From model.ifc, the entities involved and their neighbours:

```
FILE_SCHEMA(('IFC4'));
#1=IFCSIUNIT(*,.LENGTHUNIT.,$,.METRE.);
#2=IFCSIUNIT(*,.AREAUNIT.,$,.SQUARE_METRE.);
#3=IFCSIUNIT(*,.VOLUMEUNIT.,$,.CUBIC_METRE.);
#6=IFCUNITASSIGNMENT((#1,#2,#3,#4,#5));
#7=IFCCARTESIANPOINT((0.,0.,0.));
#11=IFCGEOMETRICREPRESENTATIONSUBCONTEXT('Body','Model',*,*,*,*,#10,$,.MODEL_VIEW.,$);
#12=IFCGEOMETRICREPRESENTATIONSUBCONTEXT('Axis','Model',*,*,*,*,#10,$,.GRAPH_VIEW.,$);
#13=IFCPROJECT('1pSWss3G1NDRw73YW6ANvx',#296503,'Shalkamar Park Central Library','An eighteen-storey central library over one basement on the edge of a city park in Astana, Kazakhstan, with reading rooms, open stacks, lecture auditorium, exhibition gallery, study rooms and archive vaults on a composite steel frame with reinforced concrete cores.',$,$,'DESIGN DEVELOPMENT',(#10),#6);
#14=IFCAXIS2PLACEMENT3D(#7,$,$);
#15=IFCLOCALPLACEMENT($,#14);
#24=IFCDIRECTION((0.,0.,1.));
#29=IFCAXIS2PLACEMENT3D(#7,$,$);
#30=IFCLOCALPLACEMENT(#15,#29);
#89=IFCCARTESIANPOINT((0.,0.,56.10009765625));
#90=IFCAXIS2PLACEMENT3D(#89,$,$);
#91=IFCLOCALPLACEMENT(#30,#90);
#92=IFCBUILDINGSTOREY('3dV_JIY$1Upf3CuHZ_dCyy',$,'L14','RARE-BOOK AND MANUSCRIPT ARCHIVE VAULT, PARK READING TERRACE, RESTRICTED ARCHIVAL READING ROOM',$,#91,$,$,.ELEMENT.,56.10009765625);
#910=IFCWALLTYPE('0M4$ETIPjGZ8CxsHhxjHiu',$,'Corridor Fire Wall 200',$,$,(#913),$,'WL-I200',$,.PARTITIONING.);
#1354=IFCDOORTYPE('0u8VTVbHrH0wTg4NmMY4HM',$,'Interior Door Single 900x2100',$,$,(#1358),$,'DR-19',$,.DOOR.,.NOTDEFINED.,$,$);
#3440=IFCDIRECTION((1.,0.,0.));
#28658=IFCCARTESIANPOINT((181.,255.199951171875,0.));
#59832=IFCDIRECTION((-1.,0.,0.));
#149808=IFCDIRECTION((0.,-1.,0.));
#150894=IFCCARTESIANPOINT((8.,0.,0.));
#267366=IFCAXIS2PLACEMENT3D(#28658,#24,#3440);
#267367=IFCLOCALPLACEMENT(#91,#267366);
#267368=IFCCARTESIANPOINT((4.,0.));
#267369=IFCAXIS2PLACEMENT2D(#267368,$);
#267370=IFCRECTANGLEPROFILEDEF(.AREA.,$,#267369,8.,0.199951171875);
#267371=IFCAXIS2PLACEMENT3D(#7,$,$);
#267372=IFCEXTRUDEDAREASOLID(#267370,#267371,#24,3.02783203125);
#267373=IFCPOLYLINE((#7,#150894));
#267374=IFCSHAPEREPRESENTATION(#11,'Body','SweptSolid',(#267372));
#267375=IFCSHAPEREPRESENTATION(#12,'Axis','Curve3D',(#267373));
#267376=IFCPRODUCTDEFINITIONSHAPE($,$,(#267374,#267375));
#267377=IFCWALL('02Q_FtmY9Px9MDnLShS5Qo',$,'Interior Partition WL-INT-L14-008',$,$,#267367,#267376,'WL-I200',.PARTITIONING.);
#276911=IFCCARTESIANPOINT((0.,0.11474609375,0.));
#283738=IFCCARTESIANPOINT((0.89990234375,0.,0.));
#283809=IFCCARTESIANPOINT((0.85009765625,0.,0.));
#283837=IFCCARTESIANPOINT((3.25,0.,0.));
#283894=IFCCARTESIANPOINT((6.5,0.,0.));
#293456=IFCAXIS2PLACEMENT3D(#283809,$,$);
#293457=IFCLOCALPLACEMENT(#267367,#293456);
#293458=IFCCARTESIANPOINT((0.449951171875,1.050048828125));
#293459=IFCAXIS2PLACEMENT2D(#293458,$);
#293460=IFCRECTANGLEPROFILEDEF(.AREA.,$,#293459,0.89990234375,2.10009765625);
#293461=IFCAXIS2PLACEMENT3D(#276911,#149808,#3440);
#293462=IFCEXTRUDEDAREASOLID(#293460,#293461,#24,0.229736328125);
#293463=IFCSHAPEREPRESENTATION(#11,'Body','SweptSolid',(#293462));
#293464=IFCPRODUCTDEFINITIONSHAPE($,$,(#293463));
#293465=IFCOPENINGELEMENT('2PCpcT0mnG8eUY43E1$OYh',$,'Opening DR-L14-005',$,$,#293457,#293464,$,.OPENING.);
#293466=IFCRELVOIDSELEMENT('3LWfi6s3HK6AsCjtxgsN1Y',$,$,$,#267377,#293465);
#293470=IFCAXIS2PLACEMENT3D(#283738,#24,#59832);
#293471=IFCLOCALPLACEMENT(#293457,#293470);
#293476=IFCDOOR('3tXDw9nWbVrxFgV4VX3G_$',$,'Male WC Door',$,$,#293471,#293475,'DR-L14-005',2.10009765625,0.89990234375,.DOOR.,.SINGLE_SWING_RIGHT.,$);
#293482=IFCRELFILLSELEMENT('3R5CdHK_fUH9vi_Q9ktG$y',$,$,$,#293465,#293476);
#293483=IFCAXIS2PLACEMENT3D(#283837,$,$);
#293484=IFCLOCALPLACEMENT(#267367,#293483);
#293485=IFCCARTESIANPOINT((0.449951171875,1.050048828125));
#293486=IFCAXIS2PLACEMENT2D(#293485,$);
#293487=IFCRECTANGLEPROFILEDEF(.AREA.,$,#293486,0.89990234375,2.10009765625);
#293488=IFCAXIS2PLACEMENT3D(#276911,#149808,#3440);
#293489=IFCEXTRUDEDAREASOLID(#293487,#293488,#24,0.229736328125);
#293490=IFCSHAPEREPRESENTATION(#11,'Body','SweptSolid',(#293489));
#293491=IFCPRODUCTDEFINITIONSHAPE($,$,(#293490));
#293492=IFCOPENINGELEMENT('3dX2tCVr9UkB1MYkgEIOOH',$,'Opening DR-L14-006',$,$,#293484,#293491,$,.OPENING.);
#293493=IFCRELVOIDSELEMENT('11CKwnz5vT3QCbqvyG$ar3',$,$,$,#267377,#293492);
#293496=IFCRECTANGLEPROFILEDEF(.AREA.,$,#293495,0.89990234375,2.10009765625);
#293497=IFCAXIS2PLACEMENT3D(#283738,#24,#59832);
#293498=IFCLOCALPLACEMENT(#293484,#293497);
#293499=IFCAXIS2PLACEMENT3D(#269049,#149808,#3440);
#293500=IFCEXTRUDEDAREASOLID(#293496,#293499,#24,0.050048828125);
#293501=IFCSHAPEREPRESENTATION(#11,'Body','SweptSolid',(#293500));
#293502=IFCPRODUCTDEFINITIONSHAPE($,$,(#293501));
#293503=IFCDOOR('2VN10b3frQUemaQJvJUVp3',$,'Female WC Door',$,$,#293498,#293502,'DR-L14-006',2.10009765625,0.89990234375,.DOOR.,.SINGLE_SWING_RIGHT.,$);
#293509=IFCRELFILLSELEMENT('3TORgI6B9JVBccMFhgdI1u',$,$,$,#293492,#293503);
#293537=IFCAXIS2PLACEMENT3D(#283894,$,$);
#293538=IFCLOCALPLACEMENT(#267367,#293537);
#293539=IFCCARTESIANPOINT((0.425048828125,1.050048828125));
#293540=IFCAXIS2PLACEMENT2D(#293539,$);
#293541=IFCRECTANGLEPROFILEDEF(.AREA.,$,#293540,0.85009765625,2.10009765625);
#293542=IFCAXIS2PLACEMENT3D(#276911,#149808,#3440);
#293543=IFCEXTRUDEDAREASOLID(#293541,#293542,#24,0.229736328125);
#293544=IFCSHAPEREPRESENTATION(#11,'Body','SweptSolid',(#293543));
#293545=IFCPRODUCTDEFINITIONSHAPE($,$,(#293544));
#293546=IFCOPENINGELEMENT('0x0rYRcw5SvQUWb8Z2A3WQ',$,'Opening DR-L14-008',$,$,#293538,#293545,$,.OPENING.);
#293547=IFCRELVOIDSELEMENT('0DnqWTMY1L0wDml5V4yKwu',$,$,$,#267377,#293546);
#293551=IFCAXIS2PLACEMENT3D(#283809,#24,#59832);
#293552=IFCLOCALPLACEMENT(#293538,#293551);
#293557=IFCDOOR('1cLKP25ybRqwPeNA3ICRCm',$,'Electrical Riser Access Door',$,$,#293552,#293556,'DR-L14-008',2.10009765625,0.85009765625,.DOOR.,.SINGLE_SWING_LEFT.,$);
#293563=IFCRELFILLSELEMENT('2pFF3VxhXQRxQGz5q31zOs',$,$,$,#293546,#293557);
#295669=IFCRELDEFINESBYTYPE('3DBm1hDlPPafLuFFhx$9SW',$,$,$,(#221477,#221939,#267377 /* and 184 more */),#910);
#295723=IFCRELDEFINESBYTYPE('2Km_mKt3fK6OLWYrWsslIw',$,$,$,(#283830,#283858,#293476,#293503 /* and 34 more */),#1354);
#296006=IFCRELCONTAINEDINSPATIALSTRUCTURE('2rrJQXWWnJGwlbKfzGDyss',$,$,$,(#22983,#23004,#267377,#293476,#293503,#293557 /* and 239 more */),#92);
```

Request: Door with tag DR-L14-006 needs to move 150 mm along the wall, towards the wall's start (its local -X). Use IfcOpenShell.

```python
import ifcopenshell
import ifcopenshell.api.geometry
import ifcopenshell.util.placement

model = ifcopenshell.open("model.ifc")

door = model.by_guid("2VN10b3frQUemaQJvJUVp3")
opening = door.FillsVoids[0].RelatingOpeningElement
wall = opening.VoidsElements[0].RelatingBuildingElement

wall_matrix = ifcopenshell.util.placement.get_local_placement(wall.ObjectPlacement)
shift = wall_matrix[:3, 0] * -0.15
before = ifcopenshell.util.placement.get_local_placement(door.ObjectPlacement)[:3, 3].copy()

# The door is placed relative to its opening, so it follows when the opening moves.
matrix = ifcopenshell.util.placement.get_local_placement(opening.ObjectPlacement)
matrix[:3, 3] += shift
ifcopenshell.api.geometry.edit_object_placement(
    model, product=opening, matrix=matrix, is_si=False, should_transform_children=True
)

after = ifcopenshell.util.placement.get_local_placement(door.ObjectPlacement)[:3, 3]
print("door moved by", (after - before).round(3) + 0.0)

model.write("model_edited.ifc")
```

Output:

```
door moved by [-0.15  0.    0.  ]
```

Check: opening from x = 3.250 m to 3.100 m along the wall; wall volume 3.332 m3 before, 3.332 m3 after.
